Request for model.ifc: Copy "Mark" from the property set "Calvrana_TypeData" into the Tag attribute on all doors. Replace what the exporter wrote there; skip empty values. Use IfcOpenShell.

First a look at what the model holds.

```python
import ifcopenshell
import ifcopenshell.util.element

model = ifcopenshell.open("model.ifc")
print(model.schema)
doors = model.by_type("IfcDoor")
print(len(doors), "doors")
for e in doors[:8]:
    source = ifcopenshell.util.element.get_pset(e, "Calvrana_TypeData", "Mark")
    target = e.Tag
    print(e.id(), repr(source), repr(target), sep=" | ")
```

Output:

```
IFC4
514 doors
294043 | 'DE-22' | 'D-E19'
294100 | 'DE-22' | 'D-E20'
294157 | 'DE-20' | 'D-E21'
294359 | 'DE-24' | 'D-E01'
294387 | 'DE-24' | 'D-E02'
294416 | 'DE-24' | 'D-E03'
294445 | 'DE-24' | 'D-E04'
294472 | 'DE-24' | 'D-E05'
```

```python
import ifcopenshell
import ifcopenshell.util.element

model = ifcopenshell.open("model.ifc")

count = 0
for e in model.by_type("IfcDoor"):
    value = ifcopenshell.util.element.get_pset(e, "Calvrana_TypeData", "Mark")
    current = e.Tag
    if not value or not value.strip() or current == value:
        continue
    e.Tag = value
    count += 1

print(count, "doors updated")

model.write("model_v2.ifc")
```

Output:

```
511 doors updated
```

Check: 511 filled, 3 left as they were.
